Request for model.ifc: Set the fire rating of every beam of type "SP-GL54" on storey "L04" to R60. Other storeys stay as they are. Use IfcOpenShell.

First a look at what the model holds.

```python
import ifcopenshell
import ifcopenshell.util.element

model = ifcopenshell.open("model.ifc")
print(model.schema)
storey = next(s for s in model.by_type("IfcBuildingStorey") if s.Name == "L04")
beams = [e for e in ifcopenshell.util.element.get_decomposition(storey) if e.is_a("IfcBeam")]
seen = {}
for e in beams:
    element_type = ifcopenshell.util.element.get_type(e)
    key = (element_type.Name if element_type != e and element_type else None, ifcopenshell.util.element.get_pset(e, "Pset_BeamCommon", "FireRating"))
    seen[key] = seen.get(key, 0) + 1
for (name, value), count in sorted(seen.items(), key=str):
    print(count, "x", name, "|", value)
```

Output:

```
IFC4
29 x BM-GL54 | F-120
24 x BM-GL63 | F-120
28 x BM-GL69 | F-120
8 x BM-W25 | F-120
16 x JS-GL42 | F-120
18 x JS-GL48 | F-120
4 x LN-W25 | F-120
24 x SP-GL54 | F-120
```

```python
import ifcopenshell
import ifcopenshell.api.pset
import ifcopenshell.util.element

model = ifcopenshell.open("model.ifc")

storey = next(s for s in model.by_type("IfcBuildingStorey") if s.Name == "L04")
beams = [e for e in ifcopenshell.util.element.get_decomposition(storey) if e.is_a("IfcBeam")]

count = 0
for e in beams:
    element_type = ifcopenshell.util.element.get_type(e)
    if element_type in (None, e) or element_type.Name != "SP-GL54":
        continue
    # add_pset returns the element's existing set when there is one.
    pset = ifcopenshell.api.pset.add_pset(model, product=e, name="Pset_BeamCommon")
    ifcopenshell.api.pset.edit_pset(model, pset=pset, properties={"FireRating": "R60"})
    count += 1

print(count, "beams updated")

model.write("model-out.ifc")
```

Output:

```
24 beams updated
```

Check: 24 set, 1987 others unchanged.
